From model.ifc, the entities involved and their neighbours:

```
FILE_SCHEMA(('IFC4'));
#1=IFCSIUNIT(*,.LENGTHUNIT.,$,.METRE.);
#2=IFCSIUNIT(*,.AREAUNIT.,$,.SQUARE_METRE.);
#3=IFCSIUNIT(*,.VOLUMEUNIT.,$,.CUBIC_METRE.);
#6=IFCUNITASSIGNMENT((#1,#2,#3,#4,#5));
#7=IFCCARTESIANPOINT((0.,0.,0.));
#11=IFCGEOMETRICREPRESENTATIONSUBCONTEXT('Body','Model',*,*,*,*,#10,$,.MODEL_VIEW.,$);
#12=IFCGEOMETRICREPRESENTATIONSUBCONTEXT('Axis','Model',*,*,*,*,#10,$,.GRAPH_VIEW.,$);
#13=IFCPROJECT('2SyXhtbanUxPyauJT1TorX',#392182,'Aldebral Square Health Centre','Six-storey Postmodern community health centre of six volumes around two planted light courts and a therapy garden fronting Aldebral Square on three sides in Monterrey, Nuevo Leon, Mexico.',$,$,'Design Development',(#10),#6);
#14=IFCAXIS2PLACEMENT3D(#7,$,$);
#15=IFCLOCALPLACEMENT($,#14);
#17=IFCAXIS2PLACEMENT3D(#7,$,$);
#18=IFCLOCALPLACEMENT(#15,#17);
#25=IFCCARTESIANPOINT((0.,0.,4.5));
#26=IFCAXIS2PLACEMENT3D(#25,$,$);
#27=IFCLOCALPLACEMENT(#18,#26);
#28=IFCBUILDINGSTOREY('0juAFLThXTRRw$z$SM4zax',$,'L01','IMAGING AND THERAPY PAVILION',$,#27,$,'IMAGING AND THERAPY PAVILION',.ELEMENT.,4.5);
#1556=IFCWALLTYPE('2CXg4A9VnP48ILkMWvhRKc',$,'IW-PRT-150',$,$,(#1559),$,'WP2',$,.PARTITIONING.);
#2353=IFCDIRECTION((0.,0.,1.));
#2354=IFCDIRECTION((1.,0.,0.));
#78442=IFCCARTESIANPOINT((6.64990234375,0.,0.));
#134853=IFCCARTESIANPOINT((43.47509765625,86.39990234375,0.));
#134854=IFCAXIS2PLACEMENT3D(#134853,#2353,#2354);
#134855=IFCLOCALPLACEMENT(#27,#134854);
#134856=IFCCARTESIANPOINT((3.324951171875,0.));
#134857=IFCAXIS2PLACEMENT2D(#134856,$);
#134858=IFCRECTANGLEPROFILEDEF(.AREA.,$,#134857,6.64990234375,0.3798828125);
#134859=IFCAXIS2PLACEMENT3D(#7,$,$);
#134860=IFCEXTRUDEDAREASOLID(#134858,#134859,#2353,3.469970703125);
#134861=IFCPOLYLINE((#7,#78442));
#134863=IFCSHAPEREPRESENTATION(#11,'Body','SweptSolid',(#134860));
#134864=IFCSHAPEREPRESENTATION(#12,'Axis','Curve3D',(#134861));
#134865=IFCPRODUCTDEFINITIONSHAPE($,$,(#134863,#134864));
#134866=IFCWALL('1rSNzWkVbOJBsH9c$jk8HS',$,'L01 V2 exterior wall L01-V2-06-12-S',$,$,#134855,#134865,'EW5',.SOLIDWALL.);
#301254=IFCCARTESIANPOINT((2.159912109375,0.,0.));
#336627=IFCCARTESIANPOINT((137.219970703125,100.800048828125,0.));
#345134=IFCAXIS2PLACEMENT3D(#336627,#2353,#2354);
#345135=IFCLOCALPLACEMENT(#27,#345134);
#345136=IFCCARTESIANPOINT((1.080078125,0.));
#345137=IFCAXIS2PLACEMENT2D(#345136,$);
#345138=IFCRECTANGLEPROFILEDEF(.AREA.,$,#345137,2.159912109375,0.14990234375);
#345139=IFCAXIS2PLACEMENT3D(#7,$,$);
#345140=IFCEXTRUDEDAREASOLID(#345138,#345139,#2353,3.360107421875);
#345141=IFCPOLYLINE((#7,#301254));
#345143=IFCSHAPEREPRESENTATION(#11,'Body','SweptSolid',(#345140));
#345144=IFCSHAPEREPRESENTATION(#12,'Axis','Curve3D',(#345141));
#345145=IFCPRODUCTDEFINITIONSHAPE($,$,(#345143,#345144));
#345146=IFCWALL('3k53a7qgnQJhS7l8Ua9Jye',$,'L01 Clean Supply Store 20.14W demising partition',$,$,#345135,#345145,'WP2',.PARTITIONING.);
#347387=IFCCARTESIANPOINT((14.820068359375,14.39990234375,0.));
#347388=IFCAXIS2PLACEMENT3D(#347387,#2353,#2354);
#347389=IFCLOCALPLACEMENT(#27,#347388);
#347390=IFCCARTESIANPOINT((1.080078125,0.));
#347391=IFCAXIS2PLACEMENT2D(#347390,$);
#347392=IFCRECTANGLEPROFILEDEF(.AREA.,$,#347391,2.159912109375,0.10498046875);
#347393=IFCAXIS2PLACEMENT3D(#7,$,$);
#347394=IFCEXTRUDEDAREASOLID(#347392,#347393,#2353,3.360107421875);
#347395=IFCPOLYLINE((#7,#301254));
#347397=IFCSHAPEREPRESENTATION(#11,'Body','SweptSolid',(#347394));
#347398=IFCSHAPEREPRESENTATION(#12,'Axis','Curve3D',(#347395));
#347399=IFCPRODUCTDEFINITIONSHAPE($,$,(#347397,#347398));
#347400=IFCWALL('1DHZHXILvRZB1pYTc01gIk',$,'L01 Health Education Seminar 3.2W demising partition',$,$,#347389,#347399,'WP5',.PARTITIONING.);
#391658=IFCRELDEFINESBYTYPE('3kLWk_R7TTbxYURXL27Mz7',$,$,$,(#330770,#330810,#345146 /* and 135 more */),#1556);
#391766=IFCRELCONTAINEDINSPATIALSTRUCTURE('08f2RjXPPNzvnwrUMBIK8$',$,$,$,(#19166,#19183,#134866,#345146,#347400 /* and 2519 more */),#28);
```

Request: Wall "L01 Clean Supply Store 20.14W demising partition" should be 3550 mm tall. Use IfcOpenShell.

```python
import ifcopenshell
import ifcopenshell.geom
import ifcopenshell.util.representation
import ifcopenshell.util.shape
import ifcopenshell.util.unit

model = ifcopenshell.open("model.ifc")
unit_scale = ifcopenshell.util.unit.calculate_unit_scale(model)
settings = ifcopenshell.geom.settings()


def volume(element):
    """Net volume in cubic metres, openings subtracted."""
    shape = ifcopenshell.geom.create_shape(settings, element)
    return ifcopenshell.util.shape.get_volume(shape.geometry)


wall = model.by_id(345146)
before = volume(wall)

body = ifcopenshell.util.representation.get_representation(wall, "Model", "Body")
solid = body.Items[0]
old_height = solid.Depth
solid.Depth = 3.55 / unit_scale
after = volume(wall)

print(f"height {old_height:g} -> {solid.Depth:g}, volume {before:.3f} -> {after:.3f} m3")

model.write("model_v2.ifc")
```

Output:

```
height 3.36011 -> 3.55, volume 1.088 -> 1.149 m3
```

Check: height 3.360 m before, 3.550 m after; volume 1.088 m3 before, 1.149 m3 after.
